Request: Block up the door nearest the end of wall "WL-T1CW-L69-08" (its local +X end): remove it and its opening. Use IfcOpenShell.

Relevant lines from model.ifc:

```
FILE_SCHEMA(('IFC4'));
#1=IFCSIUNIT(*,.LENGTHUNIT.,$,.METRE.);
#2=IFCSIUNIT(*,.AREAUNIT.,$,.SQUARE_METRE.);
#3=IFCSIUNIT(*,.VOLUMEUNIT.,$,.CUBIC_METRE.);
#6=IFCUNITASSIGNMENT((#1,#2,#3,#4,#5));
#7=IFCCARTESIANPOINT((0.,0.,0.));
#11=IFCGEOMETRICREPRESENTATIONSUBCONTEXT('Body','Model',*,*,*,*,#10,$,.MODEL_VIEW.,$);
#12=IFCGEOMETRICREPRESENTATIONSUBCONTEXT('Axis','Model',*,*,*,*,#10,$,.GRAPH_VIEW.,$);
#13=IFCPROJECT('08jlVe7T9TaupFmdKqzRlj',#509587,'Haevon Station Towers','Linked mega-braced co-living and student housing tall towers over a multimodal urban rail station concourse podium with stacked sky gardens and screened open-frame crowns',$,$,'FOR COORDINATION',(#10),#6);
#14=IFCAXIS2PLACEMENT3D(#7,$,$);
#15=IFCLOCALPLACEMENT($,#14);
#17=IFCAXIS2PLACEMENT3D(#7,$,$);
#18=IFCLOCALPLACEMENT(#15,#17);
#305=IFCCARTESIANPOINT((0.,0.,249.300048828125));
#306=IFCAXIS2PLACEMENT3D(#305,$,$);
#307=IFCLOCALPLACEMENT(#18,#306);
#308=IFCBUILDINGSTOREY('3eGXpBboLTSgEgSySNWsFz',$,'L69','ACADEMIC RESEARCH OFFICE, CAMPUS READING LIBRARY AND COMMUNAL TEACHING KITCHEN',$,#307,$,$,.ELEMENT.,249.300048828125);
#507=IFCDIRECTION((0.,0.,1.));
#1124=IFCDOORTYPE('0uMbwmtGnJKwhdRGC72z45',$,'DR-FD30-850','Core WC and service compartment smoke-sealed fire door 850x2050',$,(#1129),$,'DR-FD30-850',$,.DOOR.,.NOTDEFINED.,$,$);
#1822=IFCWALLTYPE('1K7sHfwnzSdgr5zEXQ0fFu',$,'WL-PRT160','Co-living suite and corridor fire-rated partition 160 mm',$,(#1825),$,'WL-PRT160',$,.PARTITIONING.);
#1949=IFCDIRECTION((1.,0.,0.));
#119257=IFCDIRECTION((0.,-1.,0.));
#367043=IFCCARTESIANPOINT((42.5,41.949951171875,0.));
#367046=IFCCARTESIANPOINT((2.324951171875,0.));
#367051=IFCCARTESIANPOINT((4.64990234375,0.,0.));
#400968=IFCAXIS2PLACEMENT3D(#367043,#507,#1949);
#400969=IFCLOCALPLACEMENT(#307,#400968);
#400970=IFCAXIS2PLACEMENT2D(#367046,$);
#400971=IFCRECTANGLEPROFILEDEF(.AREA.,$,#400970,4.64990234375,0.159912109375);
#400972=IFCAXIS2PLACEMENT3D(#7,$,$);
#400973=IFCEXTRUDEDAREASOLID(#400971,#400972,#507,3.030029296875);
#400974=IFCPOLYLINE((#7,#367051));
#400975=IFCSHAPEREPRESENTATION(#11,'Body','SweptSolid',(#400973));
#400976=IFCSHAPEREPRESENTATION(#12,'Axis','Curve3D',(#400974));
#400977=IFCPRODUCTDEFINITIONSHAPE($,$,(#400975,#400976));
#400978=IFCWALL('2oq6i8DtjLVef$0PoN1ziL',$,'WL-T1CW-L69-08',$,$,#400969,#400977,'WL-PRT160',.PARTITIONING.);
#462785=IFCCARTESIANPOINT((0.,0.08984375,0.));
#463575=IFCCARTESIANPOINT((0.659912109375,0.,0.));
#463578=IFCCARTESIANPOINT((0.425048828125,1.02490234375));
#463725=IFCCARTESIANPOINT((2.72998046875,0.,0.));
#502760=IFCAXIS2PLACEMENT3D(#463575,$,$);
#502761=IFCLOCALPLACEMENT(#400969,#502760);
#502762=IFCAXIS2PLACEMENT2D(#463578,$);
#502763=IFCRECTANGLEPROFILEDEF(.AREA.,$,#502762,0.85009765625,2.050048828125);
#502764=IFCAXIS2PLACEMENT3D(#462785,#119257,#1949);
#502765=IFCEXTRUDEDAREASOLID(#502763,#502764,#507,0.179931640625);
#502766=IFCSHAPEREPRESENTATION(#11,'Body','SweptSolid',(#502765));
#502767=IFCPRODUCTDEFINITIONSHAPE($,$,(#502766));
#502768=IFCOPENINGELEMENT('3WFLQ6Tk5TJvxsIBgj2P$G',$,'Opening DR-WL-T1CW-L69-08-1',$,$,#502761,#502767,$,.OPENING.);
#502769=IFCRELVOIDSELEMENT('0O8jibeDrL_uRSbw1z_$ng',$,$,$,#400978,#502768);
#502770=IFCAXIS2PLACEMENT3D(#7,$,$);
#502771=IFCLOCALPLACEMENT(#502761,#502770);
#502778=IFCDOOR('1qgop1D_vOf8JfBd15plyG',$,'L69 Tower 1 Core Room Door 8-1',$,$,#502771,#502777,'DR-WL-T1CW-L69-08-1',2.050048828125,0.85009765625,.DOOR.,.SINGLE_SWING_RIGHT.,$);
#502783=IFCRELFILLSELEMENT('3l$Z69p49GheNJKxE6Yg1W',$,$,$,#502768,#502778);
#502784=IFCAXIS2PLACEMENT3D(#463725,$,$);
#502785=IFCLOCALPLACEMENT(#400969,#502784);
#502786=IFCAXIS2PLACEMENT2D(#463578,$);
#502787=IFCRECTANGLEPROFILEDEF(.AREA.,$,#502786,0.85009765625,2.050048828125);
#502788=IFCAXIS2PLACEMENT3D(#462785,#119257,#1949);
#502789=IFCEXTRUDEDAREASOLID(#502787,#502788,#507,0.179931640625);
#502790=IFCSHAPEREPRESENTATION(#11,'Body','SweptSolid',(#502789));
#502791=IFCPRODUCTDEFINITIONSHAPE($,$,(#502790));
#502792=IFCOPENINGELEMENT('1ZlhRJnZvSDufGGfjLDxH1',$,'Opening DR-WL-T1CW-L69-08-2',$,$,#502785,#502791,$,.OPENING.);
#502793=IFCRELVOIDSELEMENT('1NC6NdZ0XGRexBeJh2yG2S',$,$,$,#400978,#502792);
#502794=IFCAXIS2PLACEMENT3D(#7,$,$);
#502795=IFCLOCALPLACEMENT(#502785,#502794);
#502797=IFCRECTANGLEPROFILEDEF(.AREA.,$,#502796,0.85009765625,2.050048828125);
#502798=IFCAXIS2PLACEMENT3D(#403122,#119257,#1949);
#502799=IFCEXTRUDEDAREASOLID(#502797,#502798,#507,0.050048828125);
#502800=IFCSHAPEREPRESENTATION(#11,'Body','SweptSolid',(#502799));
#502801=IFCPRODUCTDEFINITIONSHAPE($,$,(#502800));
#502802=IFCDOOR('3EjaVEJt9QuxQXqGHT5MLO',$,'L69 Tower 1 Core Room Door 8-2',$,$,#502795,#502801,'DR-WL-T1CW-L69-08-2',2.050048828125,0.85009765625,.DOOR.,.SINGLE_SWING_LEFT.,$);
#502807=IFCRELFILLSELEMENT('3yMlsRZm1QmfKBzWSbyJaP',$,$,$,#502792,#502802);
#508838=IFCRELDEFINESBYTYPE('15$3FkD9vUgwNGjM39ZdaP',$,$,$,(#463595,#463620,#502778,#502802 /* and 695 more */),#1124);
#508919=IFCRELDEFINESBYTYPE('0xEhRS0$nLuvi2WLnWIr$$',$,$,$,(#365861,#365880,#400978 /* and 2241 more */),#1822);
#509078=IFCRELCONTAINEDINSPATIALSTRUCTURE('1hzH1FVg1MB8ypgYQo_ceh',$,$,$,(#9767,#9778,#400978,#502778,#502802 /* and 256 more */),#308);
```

```python
import ifcopenshell
import ifcopenshell.api.feature
import ifcopenshell.api.root
import ifcopenshell.geom
import ifcopenshell.util.shape

model = ifcopenshell.open("model.ifc")
settings = ifcopenshell.geom.settings()


def volume(element):
    """Net volume in cubic metres, openings subtracted."""
    shape = ifcopenshell.geom.create_shape(settings, element)
    return ifcopenshell.util.shape.get_volume(shape.geometry)


door = model.by_guid("3EjaVEJt9QuxQXqGHT5MLO")
opening = door.FillsVoids[0].RelatingOpeningElement
wall = opening.VoidsElements[0].RelatingBuildingElement
before = volume(wall)

ifcopenshell.api.root.remove_product(model, product=door)
ifcopenshell.api.feature.remove_feature(model, feature=opening)

after = volume(wall)

print(f"wall volume {before:.3f} -> {after:.3f} m3")

model.write("model_updated.ifc")
```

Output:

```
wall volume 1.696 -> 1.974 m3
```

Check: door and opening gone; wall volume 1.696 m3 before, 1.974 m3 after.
